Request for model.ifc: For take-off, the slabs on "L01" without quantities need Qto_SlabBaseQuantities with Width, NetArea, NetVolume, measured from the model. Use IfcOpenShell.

First a look at what the model holds.

```python
import ifcopenshell
import ifcopenshell.util.element
import ifcopenshell.util.unit

model = ifcopenshell.open("model.ifc")
print(model.schema)
for unit_type in ("LENGTHUNIT", "AREAUNIT", "VOLUMEUNIT"):
    print(unit_type, ifcopenshell.util.unit.calculate_unit_scale(model, unit_type))
storey = next(s for s in model.by_type("IfcBuildingStorey") if s.Name == "L01")
slabs = [e for e in ifcopenshell.util.element.get_decomposition(storey) if e.is_a("IfcSlab")]
for e in sorted(slabs, key=lambda e: e.id()):
    print(e.id(), e.is_a(), e.Name, list(ifcopenshell.util.element.get_psets(e, qtos_only=True)), sep=" | ")
```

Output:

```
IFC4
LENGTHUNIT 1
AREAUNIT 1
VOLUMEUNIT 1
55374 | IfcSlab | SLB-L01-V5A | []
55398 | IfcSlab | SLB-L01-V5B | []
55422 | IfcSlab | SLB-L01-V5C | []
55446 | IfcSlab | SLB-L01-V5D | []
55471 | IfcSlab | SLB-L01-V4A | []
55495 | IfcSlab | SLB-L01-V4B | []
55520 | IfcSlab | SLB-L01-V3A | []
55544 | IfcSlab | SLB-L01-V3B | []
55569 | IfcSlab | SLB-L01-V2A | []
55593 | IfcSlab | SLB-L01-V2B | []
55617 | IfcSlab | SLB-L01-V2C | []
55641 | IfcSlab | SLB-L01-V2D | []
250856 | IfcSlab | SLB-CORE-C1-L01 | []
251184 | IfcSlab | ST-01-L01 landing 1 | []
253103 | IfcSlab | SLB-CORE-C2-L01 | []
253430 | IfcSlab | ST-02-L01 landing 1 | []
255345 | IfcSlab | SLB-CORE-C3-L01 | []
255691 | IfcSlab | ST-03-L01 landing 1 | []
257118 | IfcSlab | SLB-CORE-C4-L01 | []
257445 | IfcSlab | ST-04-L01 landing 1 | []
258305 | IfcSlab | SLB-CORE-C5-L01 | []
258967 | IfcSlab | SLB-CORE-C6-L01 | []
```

```python
import ifcopenshell
import ifcopenshell.api.pset
import ifcopenshell.geom
import ifcopenshell.util.element
import ifcopenshell.util.shape
import ifcopenshell.util.unit

model = ifcopenshell.open("model.ifc")
unit_scale = ifcopenshell.util.unit.calculate_unit_scale(model)
area_scale = ifcopenshell.util.unit.calculate_unit_scale(model, "AREAUNIT")
volume_scale = ifcopenshell.util.unit.calculate_unit_scale(model, "VOLUMEUNIT")
settings = ifcopenshell.geom.settings()

storey = next(s for s in model.by_type("IfcBuildingStorey") if s.Name == "L01")
slabs = [e for e in ifcopenshell.util.element.get_decomposition(storey) if e.is_a("IfcSlab")]

for e in sorted(slabs, key=lambda e: e.id()):
    if ifcopenshell.util.element.get_psets(e, qtos_only=True, should_inherit=False):
        continue
    # Geometry comes back in metres, in the element's own axes.
    shape = ifcopenshell.geom.create_shape(settings, e)
    values = {
        "Width": ifcopenshell.util.shape.get_z(shape.geometry) / unit_scale,
        "NetArea": ifcopenshell.util.shape.get_footprint_area(shape.geometry) / area_scale,
        "NetVolume": ifcopenshell.util.shape.get_volume(shape.geometry) / volume_scale,
    }
    qto = ifcopenshell.api.pset.add_qto(model, product=e, name="Qto_SlabBaseQuantities")
    ifcopenshell.api.pset.edit_qto(model, qto=qto, properties=values)
    print(e.id(), {k: round(v, 3) for k, v in values.items()})

model.write("model-out.ifc")
```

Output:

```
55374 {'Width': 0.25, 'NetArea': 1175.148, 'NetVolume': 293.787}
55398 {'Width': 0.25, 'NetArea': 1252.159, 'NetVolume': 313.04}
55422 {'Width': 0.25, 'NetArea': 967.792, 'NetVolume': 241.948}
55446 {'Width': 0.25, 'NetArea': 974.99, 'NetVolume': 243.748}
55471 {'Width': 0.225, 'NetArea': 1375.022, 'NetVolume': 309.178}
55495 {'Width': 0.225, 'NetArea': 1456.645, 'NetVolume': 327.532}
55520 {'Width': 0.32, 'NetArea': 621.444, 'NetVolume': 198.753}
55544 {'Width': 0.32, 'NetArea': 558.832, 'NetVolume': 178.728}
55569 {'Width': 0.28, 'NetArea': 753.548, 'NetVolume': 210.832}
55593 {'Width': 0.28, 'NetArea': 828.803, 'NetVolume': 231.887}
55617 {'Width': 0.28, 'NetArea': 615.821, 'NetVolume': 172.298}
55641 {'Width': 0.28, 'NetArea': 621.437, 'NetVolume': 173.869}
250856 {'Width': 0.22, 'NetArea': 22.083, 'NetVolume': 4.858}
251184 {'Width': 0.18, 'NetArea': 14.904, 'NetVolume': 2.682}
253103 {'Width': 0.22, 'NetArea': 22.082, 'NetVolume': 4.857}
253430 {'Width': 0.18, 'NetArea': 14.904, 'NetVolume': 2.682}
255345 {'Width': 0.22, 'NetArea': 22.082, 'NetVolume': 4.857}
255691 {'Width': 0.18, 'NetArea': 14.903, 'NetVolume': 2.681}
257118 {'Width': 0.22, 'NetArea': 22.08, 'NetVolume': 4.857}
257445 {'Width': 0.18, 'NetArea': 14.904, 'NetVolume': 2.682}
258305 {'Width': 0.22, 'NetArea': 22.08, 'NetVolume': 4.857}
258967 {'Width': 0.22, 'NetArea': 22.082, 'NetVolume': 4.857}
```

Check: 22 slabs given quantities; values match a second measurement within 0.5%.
